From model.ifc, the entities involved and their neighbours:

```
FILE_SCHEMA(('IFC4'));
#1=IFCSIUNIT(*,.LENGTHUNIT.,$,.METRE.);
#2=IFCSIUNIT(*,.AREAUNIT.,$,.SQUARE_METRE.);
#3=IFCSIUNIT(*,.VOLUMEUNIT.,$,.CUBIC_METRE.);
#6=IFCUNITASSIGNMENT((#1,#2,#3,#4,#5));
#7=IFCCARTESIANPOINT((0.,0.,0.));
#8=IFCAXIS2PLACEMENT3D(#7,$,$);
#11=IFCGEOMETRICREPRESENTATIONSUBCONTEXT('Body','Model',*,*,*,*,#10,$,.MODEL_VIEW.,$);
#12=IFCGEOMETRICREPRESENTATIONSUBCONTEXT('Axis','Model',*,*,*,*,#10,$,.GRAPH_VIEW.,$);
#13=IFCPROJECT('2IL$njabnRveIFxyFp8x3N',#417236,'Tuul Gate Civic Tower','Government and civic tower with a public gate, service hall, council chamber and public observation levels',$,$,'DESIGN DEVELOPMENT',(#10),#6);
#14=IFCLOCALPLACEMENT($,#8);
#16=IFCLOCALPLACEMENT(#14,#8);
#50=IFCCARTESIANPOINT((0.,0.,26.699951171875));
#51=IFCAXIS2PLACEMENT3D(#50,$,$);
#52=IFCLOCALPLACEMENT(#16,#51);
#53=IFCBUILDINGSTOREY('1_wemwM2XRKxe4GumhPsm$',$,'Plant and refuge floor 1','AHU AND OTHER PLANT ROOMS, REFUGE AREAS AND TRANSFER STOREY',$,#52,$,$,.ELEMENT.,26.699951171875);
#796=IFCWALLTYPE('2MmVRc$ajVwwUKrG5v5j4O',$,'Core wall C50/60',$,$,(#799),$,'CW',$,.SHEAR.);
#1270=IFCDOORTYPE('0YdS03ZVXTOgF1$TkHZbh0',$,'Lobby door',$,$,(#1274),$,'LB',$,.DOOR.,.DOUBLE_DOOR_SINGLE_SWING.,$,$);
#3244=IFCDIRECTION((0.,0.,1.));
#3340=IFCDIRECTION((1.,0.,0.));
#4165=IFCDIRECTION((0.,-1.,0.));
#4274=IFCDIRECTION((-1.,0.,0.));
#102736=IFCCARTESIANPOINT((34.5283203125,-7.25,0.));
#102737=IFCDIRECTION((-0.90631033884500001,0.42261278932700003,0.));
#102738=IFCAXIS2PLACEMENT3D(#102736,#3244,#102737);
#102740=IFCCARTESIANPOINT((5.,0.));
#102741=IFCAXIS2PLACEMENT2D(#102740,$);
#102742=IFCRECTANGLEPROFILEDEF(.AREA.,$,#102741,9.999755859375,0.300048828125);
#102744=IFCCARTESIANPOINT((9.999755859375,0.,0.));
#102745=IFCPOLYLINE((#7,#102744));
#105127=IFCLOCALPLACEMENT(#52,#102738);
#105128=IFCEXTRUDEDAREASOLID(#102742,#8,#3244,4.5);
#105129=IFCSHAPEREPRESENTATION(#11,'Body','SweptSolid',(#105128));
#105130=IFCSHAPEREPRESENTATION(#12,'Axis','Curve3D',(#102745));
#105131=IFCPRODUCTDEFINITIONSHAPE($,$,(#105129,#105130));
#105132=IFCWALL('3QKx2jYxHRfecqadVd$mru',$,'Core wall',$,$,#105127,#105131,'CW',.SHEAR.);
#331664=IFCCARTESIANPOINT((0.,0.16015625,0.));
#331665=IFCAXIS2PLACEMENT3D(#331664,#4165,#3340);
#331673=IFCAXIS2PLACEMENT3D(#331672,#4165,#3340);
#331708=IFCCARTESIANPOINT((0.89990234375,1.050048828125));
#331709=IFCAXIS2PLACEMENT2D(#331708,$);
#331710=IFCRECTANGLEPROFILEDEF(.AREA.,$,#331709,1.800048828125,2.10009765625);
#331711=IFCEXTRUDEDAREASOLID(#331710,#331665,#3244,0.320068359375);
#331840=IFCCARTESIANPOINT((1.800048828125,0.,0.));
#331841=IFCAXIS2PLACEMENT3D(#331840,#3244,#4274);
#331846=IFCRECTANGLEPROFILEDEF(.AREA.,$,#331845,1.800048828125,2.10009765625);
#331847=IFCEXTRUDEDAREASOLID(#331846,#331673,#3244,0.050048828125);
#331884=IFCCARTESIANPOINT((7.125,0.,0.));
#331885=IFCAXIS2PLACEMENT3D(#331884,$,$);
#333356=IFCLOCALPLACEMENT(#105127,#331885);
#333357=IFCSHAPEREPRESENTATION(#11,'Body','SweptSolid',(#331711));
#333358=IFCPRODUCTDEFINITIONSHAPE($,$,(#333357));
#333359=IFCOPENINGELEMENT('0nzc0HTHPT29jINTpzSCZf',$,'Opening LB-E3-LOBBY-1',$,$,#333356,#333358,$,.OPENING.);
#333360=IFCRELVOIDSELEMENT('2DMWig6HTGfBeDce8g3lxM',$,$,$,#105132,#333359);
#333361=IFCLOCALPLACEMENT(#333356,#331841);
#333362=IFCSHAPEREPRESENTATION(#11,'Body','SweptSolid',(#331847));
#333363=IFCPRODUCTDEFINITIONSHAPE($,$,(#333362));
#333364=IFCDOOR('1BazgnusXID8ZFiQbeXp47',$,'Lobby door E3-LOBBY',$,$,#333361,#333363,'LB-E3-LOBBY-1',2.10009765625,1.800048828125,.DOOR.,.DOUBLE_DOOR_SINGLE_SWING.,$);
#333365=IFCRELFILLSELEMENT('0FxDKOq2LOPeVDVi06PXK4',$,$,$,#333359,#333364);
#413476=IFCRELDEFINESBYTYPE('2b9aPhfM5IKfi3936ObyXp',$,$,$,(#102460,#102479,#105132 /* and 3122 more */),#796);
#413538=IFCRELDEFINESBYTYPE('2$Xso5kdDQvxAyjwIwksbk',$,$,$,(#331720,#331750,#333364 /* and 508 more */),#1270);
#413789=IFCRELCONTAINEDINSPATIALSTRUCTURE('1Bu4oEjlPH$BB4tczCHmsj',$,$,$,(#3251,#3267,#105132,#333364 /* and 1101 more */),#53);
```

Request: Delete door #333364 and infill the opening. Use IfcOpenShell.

```python
import ifcopenshell
import ifcopenshell.api.feature
import ifcopenshell.api.root
import ifcopenshell.geom
import ifcopenshell.util.shape

model = ifcopenshell.open("model.ifc")
settings = ifcopenshell.geom.settings()


def volume(element):
    """Net volume in cubic metres, openings subtracted."""
    shape = ifcopenshell.geom.create_shape(settings, element)
    return ifcopenshell.util.shape.get_volume(shape.geometry)


door = model.by_guid("1BazgnusXID8ZFiQbeXp47")
opening = door.FillsVoids[0].RelatingOpeningElement
wall = opening.VoidsElements[0].RelatingBuildingElement
before = volume(wall)

ifcopenshell.api.root.remove_product(model, product=door)
ifcopenshell.api.feature.remove_feature(model, feature=opening)

after = volume(wall)

print(f"wall volume {before:.3f} -> {after:.3f} m3")

model.write("model-out.ifc")
```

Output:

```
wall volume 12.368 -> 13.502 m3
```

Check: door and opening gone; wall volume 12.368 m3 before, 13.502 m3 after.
